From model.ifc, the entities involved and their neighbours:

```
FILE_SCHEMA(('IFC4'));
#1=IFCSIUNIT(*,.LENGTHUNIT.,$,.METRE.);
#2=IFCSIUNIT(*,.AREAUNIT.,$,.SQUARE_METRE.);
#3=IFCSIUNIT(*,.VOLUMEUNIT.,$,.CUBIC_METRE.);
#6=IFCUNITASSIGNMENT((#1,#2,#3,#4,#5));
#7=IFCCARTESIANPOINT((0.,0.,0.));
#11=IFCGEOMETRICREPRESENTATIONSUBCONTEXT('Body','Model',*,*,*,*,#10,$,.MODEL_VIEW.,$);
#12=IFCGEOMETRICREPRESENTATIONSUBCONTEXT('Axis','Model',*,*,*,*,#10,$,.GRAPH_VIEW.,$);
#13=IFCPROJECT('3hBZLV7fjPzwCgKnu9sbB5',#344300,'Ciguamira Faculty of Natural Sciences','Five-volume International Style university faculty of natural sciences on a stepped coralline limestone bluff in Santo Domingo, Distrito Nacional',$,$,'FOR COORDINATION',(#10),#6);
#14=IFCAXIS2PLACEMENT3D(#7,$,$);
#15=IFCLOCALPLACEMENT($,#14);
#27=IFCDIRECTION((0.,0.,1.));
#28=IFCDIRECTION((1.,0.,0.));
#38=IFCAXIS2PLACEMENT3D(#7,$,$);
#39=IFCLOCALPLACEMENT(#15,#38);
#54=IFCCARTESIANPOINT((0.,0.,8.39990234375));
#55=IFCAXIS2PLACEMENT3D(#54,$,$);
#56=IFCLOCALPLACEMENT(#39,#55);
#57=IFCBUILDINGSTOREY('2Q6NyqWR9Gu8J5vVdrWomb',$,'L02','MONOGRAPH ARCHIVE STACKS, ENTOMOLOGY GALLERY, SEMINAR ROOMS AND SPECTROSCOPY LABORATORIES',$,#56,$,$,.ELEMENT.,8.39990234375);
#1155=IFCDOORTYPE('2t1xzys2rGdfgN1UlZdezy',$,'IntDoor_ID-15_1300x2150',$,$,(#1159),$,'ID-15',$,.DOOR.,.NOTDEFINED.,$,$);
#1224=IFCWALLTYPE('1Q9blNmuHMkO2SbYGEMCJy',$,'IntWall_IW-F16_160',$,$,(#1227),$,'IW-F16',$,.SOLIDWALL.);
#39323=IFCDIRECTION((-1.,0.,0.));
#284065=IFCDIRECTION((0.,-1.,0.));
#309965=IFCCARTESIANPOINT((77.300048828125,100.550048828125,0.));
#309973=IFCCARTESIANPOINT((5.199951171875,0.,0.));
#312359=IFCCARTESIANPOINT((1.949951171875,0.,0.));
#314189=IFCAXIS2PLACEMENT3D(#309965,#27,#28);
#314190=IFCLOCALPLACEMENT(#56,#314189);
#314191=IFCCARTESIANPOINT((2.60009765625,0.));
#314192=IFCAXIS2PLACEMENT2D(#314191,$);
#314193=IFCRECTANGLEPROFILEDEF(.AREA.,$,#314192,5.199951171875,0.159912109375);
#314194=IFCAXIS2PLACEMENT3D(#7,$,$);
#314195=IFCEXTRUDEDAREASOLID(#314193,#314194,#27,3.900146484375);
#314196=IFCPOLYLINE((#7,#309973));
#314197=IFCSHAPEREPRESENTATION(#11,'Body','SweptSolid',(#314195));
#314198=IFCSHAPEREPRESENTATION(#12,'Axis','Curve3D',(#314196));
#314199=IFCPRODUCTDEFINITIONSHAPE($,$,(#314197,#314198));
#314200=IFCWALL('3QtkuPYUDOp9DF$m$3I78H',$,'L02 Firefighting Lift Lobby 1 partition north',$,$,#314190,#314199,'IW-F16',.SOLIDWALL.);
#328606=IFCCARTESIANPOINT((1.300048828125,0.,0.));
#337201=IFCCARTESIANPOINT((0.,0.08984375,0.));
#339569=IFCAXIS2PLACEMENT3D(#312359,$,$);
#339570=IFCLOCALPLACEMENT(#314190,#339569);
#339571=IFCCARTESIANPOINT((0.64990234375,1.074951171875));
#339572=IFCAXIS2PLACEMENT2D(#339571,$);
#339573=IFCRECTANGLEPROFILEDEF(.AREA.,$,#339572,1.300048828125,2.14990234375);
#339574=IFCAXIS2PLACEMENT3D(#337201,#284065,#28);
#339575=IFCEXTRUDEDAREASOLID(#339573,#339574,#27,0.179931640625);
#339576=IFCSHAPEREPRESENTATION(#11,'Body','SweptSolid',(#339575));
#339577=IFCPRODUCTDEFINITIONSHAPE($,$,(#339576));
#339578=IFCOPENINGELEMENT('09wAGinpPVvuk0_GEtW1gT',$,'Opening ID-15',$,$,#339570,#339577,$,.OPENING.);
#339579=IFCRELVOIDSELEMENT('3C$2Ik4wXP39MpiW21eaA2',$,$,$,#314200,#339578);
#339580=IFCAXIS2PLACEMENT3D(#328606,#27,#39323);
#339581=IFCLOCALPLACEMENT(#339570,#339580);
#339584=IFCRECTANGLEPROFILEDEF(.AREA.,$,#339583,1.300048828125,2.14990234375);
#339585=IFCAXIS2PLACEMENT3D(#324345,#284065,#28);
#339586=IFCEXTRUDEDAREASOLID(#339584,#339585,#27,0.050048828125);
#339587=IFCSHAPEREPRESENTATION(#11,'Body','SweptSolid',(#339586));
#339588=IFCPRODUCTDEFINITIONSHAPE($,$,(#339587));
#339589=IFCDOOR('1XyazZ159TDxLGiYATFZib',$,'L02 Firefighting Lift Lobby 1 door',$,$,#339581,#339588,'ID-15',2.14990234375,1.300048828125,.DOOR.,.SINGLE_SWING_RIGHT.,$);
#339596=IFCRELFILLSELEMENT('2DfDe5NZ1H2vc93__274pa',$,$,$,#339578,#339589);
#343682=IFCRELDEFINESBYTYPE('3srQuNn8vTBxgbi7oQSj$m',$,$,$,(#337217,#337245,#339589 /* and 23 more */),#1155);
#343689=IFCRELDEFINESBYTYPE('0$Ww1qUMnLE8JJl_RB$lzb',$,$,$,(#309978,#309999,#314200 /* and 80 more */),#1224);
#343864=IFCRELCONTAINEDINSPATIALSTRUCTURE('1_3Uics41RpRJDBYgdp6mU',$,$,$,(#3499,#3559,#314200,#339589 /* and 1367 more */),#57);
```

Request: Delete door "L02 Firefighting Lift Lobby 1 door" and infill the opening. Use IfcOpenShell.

```python
import ifcopenshell
import ifcopenshell.api.feature
import ifcopenshell.api.root
import ifcopenshell.geom
import ifcopenshell.util.shape

model = ifcopenshell.open("model.ifc")
settings = ifcopenshell.geom.settings()


def volume(element):
    """Net volume in cubic metres, openings subtracted."""
    shape = ifcopenshell.geom.create_shape(settings, element)
    return ifcopenshell.util.shape.get_volume(shape.geometry)


door = model.by_guid("1XyazZ159TDxLGiYATFZib")
opening = door.FillsVoids[0].RelatingOpeningElement
wall = opening.VoidsElements[0].RelatingBuildingElement
before = volume(wall)

ifcopenshell.api.root.remove_product(model, product=door)
ifcopenshell.api.feature.remove_feature(model, feature=opening)

after = volume(wall)

print(f"wall volume {before:.3f} -> {after:.3f} m3")

model.write("model_updated.ifc")
```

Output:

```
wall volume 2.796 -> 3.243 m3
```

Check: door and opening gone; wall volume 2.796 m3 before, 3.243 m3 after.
